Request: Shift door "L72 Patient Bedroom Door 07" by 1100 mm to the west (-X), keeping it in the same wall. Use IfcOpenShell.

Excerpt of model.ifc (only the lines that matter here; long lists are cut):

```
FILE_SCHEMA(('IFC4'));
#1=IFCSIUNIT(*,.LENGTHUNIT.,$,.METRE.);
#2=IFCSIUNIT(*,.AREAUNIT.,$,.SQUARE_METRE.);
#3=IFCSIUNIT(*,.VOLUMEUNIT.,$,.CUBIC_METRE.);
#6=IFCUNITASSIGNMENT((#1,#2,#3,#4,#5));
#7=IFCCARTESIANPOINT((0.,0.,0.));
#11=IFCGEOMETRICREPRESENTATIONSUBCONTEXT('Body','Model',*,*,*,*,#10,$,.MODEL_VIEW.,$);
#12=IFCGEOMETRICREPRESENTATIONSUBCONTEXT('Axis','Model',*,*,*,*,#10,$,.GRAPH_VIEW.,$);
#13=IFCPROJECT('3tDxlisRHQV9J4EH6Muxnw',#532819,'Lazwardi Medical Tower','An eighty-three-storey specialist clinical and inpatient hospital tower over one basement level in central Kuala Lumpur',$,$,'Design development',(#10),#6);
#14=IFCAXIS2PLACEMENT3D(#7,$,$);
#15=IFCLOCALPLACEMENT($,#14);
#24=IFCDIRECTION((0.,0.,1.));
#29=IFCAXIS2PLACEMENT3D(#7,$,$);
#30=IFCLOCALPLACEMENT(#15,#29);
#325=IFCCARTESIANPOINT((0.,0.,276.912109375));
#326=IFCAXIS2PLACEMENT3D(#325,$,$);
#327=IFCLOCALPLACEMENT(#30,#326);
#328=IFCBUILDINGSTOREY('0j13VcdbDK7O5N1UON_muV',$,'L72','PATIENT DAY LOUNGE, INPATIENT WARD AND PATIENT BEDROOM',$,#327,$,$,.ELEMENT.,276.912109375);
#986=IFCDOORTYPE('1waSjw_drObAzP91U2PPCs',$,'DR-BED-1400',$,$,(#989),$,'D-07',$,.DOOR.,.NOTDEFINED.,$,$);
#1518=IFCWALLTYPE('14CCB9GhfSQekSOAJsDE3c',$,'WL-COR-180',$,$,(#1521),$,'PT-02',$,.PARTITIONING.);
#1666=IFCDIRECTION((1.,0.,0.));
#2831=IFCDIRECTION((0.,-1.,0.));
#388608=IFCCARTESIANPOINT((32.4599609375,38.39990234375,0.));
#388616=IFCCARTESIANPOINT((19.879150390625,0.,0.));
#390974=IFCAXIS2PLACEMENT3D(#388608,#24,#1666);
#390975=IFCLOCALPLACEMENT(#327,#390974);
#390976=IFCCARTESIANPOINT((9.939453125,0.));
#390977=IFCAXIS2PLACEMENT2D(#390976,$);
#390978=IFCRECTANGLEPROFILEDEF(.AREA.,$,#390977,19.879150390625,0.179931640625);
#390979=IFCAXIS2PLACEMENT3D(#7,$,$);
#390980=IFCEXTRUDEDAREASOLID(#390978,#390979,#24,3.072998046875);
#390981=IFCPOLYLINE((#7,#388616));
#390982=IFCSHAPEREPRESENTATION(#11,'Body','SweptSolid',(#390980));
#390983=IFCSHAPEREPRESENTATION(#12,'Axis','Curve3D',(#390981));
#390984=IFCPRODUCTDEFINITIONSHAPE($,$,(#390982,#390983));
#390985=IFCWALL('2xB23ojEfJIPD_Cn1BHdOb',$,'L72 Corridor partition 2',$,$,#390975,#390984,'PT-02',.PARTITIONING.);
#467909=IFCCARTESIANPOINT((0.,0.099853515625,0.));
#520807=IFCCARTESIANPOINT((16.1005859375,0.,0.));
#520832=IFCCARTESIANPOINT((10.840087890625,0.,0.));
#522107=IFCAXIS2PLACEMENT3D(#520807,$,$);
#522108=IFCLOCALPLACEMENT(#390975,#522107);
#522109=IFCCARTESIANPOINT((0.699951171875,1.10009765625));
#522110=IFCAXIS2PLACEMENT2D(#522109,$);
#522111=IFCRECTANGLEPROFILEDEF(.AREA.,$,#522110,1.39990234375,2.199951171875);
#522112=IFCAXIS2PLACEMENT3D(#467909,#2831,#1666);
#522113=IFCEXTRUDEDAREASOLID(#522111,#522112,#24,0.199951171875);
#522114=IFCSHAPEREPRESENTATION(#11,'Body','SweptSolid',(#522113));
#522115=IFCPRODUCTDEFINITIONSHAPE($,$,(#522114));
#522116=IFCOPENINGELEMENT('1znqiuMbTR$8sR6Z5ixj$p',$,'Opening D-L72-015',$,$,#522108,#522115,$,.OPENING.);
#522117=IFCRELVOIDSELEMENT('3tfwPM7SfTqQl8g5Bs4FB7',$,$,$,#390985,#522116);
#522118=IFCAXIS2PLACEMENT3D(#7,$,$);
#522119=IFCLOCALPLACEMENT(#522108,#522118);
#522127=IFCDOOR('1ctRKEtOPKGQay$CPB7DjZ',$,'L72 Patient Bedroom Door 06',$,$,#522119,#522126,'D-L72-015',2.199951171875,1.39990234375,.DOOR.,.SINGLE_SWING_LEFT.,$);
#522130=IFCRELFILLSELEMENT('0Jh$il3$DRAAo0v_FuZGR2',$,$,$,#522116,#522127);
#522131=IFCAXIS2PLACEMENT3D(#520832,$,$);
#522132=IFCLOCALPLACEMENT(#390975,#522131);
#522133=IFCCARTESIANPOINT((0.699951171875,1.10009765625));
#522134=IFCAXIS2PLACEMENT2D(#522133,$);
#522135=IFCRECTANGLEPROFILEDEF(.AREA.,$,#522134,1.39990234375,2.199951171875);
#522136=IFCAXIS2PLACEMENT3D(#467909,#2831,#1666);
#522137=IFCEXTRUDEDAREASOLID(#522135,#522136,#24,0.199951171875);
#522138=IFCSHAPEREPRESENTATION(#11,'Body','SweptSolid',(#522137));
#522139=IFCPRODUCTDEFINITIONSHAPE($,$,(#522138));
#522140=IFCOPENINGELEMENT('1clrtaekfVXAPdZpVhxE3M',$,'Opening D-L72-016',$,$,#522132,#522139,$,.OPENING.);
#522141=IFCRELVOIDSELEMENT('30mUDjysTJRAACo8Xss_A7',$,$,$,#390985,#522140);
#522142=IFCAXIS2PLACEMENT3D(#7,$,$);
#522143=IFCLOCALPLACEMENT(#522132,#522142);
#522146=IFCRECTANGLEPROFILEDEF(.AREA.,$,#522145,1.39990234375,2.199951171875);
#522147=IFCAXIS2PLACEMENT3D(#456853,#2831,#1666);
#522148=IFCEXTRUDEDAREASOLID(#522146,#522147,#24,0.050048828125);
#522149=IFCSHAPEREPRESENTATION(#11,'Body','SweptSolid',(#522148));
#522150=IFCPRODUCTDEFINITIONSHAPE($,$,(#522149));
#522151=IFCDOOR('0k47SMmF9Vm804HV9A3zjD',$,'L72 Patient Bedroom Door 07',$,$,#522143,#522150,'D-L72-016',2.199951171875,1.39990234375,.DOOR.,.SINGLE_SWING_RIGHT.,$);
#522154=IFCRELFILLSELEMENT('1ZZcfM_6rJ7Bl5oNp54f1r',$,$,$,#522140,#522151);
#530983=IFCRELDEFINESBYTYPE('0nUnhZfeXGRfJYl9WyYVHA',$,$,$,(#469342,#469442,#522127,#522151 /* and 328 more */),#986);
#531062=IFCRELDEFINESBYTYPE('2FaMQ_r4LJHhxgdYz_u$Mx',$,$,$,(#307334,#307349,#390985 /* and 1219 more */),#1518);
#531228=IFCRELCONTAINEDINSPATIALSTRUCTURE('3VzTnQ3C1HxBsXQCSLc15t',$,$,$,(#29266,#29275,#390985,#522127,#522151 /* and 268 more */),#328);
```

```python
import ifcopenshell
import ifcopenshell.api.geometry
import ifcopenshell.util.placement

model = ifcopenshell.open("model.ifc")

door = model.by_guid("0k47SMmF9Vm804HV9A3zjD")
opening = door.FillsVoids[0].RelatingOpeningElement
wall = opening.VoidsElements[0].RelatingBuildingElement

wall_matrix = ifcopenshell.util.placement.get_local_placement(wall.ObjectPlacement)
shift = wall_matrix[:3, 0] * -1.1
before = ifcopenshell.util.placement.get_local_placement(door.ObjectPlacement)[:3, 3].copy()

# The door is placed relative to its opening, so it follows when the opening moves.
matrix = ifcopenshell.util.placement.get_local_placement(opening.ObjectPlacement)
matrix[:3, 3] += shift
ifcopenshell.api.geometry.edit_object_placement(
    model, product=opening, matrix=matrix, is_si=False, should_transform_children=True
)

after = ifcopenshell.util.placement.get_local_placement(door.ObjectPlacement)[:3, 3]
print("door moved by", (after - before).round(3) + 0.0)

model.write("model_v2.ifc")
```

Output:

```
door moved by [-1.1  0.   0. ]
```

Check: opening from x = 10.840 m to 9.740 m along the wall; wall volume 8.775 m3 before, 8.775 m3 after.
